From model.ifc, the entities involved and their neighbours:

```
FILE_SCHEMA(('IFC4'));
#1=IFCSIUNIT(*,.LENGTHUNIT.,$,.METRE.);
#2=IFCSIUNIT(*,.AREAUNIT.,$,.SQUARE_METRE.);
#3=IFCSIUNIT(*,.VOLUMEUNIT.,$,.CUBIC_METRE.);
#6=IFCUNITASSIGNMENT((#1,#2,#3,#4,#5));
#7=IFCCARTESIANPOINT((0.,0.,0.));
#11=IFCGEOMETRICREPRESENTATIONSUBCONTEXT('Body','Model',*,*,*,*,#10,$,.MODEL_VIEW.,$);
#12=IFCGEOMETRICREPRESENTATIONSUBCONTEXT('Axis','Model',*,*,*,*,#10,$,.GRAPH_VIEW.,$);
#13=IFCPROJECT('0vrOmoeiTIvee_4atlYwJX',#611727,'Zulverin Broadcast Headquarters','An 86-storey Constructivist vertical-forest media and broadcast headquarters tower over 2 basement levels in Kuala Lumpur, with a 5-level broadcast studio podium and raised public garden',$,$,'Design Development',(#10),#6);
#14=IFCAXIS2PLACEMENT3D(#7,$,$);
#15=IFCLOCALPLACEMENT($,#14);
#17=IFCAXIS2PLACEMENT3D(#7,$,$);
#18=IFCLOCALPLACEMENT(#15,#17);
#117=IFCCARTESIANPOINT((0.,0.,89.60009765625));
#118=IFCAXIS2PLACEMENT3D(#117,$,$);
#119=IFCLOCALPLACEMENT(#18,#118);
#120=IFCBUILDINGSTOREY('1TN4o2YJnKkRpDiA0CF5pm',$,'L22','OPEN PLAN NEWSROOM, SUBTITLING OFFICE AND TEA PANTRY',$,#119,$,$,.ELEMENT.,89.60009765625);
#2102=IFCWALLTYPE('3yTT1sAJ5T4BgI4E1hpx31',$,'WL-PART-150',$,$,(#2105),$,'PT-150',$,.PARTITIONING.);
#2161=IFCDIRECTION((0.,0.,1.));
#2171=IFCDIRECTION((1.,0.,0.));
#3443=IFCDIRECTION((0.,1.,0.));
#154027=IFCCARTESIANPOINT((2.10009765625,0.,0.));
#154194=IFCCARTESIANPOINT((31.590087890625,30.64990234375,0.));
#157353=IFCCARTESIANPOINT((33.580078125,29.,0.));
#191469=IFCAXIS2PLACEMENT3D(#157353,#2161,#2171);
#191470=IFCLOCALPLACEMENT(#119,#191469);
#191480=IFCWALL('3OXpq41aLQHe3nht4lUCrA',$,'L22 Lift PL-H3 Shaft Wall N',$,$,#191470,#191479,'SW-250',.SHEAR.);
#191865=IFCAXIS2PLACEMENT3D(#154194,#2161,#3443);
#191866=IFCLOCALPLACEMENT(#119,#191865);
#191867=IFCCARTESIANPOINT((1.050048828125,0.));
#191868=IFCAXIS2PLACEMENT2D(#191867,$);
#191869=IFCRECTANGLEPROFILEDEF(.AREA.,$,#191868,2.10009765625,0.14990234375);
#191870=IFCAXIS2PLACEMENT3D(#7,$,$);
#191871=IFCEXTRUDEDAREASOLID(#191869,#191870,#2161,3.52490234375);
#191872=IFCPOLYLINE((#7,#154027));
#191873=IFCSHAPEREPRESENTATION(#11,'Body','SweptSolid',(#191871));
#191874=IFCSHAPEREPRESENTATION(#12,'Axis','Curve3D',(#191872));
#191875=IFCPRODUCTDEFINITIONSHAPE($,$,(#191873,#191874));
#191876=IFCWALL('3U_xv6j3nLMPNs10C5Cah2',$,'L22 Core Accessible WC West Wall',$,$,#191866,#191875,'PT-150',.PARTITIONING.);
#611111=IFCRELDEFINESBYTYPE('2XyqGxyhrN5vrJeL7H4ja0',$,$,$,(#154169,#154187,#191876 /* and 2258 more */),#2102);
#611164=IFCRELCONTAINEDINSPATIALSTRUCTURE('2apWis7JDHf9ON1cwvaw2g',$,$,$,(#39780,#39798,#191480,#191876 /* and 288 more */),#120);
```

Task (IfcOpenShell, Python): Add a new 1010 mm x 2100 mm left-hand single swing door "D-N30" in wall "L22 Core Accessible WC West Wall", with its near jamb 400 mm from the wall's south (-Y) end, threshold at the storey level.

```python
import numpy as np
import ifcopenshell
import ifcopenshell.api.feature
import ifcopenshell.api.geometry
import ifcopenshell.api.root
import ifcopenshell.api.spatial
import ifcopenshell.geom
import ifcopenshell.util.element
import ifcopenshell.util.placement
import ifcopenshell.util.representation
import ifcopenshell.util.shape
import ifcopenshell.util.unit

model = ifcopenshell.open("model.ifc")
unit_scale = ifcopenshell.util.unit.calculate_unit_scale(model)
settings = ifcopenshell.geom.settings()


def volume(element):
    """Net volume in cubic metres, openings subtracted."""
    shape = ifcopenshell.geom.create_shape(settings, element)
    return ifcopenshell.util.shape.get_volume(shape.geometry)


wall = model.by_guid("3U_xv6j3nLMPNs10C5Cah2")
storey = ifcopenshell.util.element.get_container(wall, ifc_class="IfcBuildingStorey")
context = ifcopenshell.util.representation.get_context(model, "Model", "Body", "MODEL_VIEW")
before = volume(wall)

width, height, from_end, sill = 1.01, 2.1, 0.4, 0.0  # metres

# The wall runs along its own X axis, and the end named is its -X end.
wall_shape = ifcopenshell.geom.create_shape(settings, wall)
x, y, z = ifcopenshell.util.shape.get_vertices(wall_shape.geometry).T
start = x.min() + from_end
face, thickness = float(y.min()), float(y.max() - y.min())
wall_matrix = ifcopenshell.util.placement.get_local_placement(wall.ObjectPlacement)
level = ifcopenshell.util.placement.get_local_placement(storey.ObjectPlacement)[2, 3]


def in_wall(x, y):
    """Placement at x, y metres in the wall's axes, at sill height."""
    matrix = wall_matrix.copy()
    matrix[:, 3] = wall_matrix @ np.array([x / unit_scale, y / unit_scale, 0.0, 1.0])
    matrix[2, 3] = level + sill / unit_scale
    return matrix


# Opening: a box that overshoots both wall faces by 50 mm.
opening = ifcopenshell.api.root.create_entity(model, ifc_class="IfcOpeningElement", predefined_type="OPENING")
box = ifcopenshell.api.geometry.add_wall_representation(
    model, context=context, length=width, height=height, thickness=thickness + 0.1
)
ifcopenshell.api.geometry.assign_representation(model, product=opening, representation=box)
ifcopenshell.api.geometry.edit_object_placement(model, product=opening, matrix=in_wall(start, face - 0.05), is_si=False)
ifcopenshell.api.feature.add_feature(model, feature=opening, element=wall)

door = ifcopenshell.api.root.create_entity(model, ifc_class="IfcDoor", name="D-N30", predefined_type="DOOR")
door.OverallWidth, door.OverallHeight = width / unit_scale, height / unit_scale
door.OperationType = "SINGLE_SWING_LEFT"
body = ifcopenshell.api.geometry.add_door_representation(
    model,
    context=context,
    overall_width=door.OverallWidth,
    overall_height=door.OverallHeight,
    operation_type="SINGLE_SWING_LEFT",
    lining_properties={"LiningDepth": thickness / unit_scale, "ThresholdDepth": thickness / unit_scale},
)
ifcopenshell.api.geometry.assign_representation(model, product=door, representation=body)
ifcopenshell.api.spatial.assign_container(model, products=[door], relating_structure=storey)
ifcopenshell.api.feature.add_filling(model, opening=opening, element=door)

# The lining spans the wall, so the door starts at the wall face.
ifcopenshell.api.geometry.edit_object_placement(model, product=door, matrix=in_wall(start, face), is_si=False)

after = volume(wall)

print(f"wall volume {before:.3f} -> {after:.3f} m3")

model.write("model_edited.ifc")
```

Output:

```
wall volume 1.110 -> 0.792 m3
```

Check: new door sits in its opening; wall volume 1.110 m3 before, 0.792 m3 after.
